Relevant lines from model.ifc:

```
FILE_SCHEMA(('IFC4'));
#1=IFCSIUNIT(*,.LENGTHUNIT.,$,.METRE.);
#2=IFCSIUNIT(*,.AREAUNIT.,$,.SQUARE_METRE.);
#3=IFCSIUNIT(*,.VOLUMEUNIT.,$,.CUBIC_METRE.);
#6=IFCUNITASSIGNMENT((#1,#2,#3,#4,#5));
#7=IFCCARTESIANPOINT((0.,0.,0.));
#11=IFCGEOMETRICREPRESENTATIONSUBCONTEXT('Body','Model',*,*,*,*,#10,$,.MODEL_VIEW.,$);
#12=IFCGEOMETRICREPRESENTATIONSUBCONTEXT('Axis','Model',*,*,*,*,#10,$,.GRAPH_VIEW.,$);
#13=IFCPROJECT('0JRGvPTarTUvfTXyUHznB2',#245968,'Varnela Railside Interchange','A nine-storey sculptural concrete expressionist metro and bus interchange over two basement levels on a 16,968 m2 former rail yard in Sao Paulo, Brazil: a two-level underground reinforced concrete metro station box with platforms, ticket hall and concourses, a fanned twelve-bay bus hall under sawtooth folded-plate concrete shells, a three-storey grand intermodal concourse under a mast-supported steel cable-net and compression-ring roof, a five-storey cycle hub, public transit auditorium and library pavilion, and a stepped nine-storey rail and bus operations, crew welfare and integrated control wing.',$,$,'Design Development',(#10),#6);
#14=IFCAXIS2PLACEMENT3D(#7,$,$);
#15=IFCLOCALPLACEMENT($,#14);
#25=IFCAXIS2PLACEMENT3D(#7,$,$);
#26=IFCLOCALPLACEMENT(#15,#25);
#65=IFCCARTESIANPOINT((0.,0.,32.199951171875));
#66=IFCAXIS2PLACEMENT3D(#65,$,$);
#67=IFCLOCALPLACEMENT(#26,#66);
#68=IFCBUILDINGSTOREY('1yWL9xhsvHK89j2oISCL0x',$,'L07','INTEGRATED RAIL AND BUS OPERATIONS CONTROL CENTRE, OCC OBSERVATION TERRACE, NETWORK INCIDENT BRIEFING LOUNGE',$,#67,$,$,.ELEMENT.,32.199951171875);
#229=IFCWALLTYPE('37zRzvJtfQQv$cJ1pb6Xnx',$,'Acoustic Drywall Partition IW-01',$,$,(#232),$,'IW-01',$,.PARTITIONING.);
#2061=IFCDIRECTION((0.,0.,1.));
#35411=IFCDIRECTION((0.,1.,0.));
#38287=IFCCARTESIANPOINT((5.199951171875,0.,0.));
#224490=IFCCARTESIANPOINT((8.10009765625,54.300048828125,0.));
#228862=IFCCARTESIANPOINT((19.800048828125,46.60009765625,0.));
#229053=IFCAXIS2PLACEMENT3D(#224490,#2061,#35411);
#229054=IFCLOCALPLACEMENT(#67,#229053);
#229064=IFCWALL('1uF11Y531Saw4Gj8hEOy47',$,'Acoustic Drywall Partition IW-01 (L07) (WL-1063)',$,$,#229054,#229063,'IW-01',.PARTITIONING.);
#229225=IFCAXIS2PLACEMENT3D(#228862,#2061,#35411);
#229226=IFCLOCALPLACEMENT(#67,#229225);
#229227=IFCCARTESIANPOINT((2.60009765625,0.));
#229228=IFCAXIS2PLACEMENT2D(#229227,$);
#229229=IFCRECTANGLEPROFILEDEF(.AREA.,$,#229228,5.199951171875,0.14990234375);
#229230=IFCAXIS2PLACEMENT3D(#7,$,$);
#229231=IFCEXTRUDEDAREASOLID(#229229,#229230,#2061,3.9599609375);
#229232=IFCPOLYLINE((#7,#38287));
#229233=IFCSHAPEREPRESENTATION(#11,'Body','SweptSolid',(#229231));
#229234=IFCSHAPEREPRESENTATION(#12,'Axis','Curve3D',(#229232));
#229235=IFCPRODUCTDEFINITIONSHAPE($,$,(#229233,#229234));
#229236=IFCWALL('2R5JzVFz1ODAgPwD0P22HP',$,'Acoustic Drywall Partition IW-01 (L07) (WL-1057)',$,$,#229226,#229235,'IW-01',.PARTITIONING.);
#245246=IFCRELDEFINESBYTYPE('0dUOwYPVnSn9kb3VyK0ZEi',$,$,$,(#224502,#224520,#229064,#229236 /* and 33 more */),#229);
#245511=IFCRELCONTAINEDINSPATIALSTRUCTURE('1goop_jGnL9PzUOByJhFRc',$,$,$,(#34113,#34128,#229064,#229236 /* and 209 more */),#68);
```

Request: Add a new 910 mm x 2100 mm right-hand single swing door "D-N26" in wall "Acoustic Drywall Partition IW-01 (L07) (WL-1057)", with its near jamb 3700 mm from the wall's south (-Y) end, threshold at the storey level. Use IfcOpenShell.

```python
import numpy as np
import ifcopenshell
import ifcopenshell.api.feature
import ifcopenshell.api.geometry
import ifcopenshell.api.root
import ifcopenshell.api.spatial
import ifcopenshell.geom
import ifcopenshell.util.element
import ifcopenshell.util.placement
import ifcopenshell.util.representation
import ifcopenshell.util.shape
import ifcopenshell.util.unit

model = ifcopenshell.open("model.ifc")
unit_scale = ifcopenshell.util.unit.calculate_unit_scale(model)
settings = ifcopenshell.geom.settings()


def volume(element):
    """Net volume in cubic metres, openings subtracted."""
    shape = ifcopenshell.geom.create_shape(settings, element)
    return ifcopenshell.util.shape.get_volume(shape.geometry)


wall = model.by_guid("2R5JzVFz1ODAgPwD0P22HP")
storey = ifcopenshell.util.element.get_container(wall, ifc_class="IfcBuildingStorey")
context = ifcopenshell.util.representation.get_context(model, "Model", "Body", "MODEL_VIEW")
before = volume(wall)

width, height, from_end, sill = 0.91, 2.1, 3.7, 0.0  # metres

# The wall runs along its own X axis, and the end named is its -X end.
wall_shape = ifcopenshell.geom.create_shape(settings, wall)
x, y, z = ifcopenshell.util.shape.get_vertices(wall_shape.geometry).T
start = x.min() + from_end
face, thickness = float(y.min()), float(y.max() - y.min())
wall_matrix = ifcopenshell.util.placement.get_local_placement(wall.ObjectPlacement)
level = ifcopenshell.util.placement.get_local_placement(storey.ObjectPlacement)[2, 3]


def in_wall(x, y):
    """Placement at x, y metres in the wall's axes, at sill height."""
    matrix = wall_matrix.copy()
    matrix[:, 3] = wall_matrix @ np.array([x / unit_scale, y / unit_scale, 0.0, 1.0])
    matrix[2, 3] = level + sill / unit_scale
    return matrix


# Opening: a box that overshoots both wall faces by 50 mm.
opening = ifcopenshell.api.root.create_entity(model, ifc_class="IfcOpeningElement", predefined_type="OPENING")
box = ifcopenshell.api.geometry.add_wall_representation(
    model, context=context, length=width, height=height, thickness=thickness + 0.1
)
ifcopenshell.api.geometry.assign_representation(model, product=opening, representation=box)
ifcopenshell.api.geometry.edit_object_placement(model, product=opening, matrix=in_wall(start, face - 0.05), is_si=False)
ifcopenshell.api.feature.add_feature(model, feature=opening, element=wall)

door = ifcopenshell.api.root.create_entity(model, ifc_class="IfcDoor", name="D-N26", predefined_type="DOOR")
door.OverallWidth, door.OverallHeight = width / unit_scale, height / unit_scale
door.OperationType = "SINGLE_SWING_RIGHT"
body = ifcopenshell.api.geometry.add_door_representation(
    model,
    context=context,
    overall_width=door.OverallWidth,
    overall_height=door.OverallHeight,
    operation_type="SINGLE_SWING_RIGHT",
    lining_properties={"LiningDepth": thickness / unit_scale, "ThresholdDepth": thickness / unit_scale},
)
ifcopenshell.api.geometry.assign_representation(model, product=door, representation=body)
ifcopenshell.api.spatial.assign_container(model, products=[door], relating_structure=storey)
ifcopenshell.api.feature.add_filling(model, opening=opening, element=door)

# The lining spans the wall, so the door starts at the wall face.
ifcopenshell.api.geometry.edit_object_placement(model, product=door, matrix=in_wall(start, face), is_si=False)

after = volume(wall)

print(f"wall volume {before:.3f} -> {after:.3f} m3")

model.write("model_updated.ifc")
```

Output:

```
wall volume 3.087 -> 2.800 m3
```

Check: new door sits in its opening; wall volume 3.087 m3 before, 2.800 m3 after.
